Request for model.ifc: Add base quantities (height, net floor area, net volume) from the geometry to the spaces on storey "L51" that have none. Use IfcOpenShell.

First a look at what the model holds.

```python
import ifcopenshell
import ifcopenshell.util.element
import ifcopenshell.util.unit

model = ifcopenshell.open("model.ifc")
print(model.schema)
for unit_type in ("LENGTHUNIT", "AREAUNIT", "VOLUMEUNIT"):
    print(unit_type, ifcopenshell.util.unit.calculate_unit_scale(model, unit_type))
storey = next(s for s in model.by_type("IfcBuildingStorey") if s.Name == "L51")
spaces = [e for e in ifcopenshell.util.element.get_decomposition(storey) if e.is_a("IfcSpace")]
for e in sorted(spaces, key=lambda e: e.id()):
    print(e.id(), e.is_a(), e.Name, list(ifcopenshell.util.element.get_psets(e, qtos_only=True)), sep=" | ")
```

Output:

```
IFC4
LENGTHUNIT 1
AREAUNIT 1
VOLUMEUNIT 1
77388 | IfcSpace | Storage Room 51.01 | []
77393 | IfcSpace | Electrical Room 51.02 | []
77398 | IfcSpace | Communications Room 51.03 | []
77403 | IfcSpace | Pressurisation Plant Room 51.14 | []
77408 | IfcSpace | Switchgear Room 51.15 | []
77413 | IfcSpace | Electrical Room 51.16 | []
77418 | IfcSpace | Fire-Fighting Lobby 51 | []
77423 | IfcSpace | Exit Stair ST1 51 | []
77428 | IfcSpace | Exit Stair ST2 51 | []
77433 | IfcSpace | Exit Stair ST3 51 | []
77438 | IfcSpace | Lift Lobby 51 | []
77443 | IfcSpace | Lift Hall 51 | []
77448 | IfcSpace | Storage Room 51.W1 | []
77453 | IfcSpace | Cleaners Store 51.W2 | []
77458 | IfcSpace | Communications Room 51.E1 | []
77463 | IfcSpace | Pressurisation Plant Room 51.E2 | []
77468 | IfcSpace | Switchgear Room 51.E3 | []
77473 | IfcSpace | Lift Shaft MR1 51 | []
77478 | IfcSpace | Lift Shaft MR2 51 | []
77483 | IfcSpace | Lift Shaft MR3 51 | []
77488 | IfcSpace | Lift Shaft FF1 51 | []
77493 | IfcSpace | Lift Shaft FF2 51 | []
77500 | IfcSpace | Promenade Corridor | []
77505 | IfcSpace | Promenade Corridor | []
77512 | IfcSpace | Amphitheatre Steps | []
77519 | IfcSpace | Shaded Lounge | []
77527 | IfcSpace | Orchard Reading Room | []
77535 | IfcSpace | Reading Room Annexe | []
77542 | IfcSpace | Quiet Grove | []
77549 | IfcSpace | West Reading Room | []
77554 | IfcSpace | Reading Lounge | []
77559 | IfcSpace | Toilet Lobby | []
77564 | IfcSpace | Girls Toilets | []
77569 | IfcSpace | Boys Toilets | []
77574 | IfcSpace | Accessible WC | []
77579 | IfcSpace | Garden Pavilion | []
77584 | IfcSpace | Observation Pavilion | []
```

```python
import ifcopenshell
import ifcopenshell.api.pset
import ifcopenshell.geom
import ifcopenshell.util.element
import ifcopenshell.util.shape
import ifcopenshell.util.unit

model = ifcopenshell.open("model.ifc")
unit_scale = ifcopenshell.util.unit.calculate_unit_scale(model)
area_scale = ifcopenshell.util.unit.calculate_unit_scale(model, "AREAUNIT")
volume_scale = ifcopenshell.util.unit.calculate_unit_scale(model, "VOLUMEUNIT")
settings = ifcopenshell.geom.settings()

storey = next(s for s in model.by_type("IfcBuildingStorey") if s.Name == "L51")
spaces = [e for e in ifcopenshell.util.element.get_decomposition(storey) if e.is_a("IfcSpace")]

for e in sorted(spaces, key=lambda e: e.id()):
    if ifcopenshell.util.element.get_psets(e, qtos_only=True, should_inherit=False):
        continue
    # Geometry comes back in metres, in the element's own axes.
    shape = ifcopenshell.geom.create_shape(settings, e)
    values = {
        "Height": ifcopenshell.util.shape.get_z(shape.geometry) / unit_scale,
        "NetFloorArea": ifcopenshell.util.shape.get_footprint_area(shape.geometry) / area_scale,
        "NetVolume": ifcopenshell.util.shape.get_volume(shape.geometry) / volume_scale,
    }
    qto = ifcopenshell.api.pset.add_qto(model, product=e, name="Qto_SpaceBaseQuantities")
    ifcopenshell.api.pset.edit_qto(model, qto=qto, properties=values)
    print(e.id(), {k: round(v, 3) for k, v in values.items()})

model.write("model_v2.ifc")
```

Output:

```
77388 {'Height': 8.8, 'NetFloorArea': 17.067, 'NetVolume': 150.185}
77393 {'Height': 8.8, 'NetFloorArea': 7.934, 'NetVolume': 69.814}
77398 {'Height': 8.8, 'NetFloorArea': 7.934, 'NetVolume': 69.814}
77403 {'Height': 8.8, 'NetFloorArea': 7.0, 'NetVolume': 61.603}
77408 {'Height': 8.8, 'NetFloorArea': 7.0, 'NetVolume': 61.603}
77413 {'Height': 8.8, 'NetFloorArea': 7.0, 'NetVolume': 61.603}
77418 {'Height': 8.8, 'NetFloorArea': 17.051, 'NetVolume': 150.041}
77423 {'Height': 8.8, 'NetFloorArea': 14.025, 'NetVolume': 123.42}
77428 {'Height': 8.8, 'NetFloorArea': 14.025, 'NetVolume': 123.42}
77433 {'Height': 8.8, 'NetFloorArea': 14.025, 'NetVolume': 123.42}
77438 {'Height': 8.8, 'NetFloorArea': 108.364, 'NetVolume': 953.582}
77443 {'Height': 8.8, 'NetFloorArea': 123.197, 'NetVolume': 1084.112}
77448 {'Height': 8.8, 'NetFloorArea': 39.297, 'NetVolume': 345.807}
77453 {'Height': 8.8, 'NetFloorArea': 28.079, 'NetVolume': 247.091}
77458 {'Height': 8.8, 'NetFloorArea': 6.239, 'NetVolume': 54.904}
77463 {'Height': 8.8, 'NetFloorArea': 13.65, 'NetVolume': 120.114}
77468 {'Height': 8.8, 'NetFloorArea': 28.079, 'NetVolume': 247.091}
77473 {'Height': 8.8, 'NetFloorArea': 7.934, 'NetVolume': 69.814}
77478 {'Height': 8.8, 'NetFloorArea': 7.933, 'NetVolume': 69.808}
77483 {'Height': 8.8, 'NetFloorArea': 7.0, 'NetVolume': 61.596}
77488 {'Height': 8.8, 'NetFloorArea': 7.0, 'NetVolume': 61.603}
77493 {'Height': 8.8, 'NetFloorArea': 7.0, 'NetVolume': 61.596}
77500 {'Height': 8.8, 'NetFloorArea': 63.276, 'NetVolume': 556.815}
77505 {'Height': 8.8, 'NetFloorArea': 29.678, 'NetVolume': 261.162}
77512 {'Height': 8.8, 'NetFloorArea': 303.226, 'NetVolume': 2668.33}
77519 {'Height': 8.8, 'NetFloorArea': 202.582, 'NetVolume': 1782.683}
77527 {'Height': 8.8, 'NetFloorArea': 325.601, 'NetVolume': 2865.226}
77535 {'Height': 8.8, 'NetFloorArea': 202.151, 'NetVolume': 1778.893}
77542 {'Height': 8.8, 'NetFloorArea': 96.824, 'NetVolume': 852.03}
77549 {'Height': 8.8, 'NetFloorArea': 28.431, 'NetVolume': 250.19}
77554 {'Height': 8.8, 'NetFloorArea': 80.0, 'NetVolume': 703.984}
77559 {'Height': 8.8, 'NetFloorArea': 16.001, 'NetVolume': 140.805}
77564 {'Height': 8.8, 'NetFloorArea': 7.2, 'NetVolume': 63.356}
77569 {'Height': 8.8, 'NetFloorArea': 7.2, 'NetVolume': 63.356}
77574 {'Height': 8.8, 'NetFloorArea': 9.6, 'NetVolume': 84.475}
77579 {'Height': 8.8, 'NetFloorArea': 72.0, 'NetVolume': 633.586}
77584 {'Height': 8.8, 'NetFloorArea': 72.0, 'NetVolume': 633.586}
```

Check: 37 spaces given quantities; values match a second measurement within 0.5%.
